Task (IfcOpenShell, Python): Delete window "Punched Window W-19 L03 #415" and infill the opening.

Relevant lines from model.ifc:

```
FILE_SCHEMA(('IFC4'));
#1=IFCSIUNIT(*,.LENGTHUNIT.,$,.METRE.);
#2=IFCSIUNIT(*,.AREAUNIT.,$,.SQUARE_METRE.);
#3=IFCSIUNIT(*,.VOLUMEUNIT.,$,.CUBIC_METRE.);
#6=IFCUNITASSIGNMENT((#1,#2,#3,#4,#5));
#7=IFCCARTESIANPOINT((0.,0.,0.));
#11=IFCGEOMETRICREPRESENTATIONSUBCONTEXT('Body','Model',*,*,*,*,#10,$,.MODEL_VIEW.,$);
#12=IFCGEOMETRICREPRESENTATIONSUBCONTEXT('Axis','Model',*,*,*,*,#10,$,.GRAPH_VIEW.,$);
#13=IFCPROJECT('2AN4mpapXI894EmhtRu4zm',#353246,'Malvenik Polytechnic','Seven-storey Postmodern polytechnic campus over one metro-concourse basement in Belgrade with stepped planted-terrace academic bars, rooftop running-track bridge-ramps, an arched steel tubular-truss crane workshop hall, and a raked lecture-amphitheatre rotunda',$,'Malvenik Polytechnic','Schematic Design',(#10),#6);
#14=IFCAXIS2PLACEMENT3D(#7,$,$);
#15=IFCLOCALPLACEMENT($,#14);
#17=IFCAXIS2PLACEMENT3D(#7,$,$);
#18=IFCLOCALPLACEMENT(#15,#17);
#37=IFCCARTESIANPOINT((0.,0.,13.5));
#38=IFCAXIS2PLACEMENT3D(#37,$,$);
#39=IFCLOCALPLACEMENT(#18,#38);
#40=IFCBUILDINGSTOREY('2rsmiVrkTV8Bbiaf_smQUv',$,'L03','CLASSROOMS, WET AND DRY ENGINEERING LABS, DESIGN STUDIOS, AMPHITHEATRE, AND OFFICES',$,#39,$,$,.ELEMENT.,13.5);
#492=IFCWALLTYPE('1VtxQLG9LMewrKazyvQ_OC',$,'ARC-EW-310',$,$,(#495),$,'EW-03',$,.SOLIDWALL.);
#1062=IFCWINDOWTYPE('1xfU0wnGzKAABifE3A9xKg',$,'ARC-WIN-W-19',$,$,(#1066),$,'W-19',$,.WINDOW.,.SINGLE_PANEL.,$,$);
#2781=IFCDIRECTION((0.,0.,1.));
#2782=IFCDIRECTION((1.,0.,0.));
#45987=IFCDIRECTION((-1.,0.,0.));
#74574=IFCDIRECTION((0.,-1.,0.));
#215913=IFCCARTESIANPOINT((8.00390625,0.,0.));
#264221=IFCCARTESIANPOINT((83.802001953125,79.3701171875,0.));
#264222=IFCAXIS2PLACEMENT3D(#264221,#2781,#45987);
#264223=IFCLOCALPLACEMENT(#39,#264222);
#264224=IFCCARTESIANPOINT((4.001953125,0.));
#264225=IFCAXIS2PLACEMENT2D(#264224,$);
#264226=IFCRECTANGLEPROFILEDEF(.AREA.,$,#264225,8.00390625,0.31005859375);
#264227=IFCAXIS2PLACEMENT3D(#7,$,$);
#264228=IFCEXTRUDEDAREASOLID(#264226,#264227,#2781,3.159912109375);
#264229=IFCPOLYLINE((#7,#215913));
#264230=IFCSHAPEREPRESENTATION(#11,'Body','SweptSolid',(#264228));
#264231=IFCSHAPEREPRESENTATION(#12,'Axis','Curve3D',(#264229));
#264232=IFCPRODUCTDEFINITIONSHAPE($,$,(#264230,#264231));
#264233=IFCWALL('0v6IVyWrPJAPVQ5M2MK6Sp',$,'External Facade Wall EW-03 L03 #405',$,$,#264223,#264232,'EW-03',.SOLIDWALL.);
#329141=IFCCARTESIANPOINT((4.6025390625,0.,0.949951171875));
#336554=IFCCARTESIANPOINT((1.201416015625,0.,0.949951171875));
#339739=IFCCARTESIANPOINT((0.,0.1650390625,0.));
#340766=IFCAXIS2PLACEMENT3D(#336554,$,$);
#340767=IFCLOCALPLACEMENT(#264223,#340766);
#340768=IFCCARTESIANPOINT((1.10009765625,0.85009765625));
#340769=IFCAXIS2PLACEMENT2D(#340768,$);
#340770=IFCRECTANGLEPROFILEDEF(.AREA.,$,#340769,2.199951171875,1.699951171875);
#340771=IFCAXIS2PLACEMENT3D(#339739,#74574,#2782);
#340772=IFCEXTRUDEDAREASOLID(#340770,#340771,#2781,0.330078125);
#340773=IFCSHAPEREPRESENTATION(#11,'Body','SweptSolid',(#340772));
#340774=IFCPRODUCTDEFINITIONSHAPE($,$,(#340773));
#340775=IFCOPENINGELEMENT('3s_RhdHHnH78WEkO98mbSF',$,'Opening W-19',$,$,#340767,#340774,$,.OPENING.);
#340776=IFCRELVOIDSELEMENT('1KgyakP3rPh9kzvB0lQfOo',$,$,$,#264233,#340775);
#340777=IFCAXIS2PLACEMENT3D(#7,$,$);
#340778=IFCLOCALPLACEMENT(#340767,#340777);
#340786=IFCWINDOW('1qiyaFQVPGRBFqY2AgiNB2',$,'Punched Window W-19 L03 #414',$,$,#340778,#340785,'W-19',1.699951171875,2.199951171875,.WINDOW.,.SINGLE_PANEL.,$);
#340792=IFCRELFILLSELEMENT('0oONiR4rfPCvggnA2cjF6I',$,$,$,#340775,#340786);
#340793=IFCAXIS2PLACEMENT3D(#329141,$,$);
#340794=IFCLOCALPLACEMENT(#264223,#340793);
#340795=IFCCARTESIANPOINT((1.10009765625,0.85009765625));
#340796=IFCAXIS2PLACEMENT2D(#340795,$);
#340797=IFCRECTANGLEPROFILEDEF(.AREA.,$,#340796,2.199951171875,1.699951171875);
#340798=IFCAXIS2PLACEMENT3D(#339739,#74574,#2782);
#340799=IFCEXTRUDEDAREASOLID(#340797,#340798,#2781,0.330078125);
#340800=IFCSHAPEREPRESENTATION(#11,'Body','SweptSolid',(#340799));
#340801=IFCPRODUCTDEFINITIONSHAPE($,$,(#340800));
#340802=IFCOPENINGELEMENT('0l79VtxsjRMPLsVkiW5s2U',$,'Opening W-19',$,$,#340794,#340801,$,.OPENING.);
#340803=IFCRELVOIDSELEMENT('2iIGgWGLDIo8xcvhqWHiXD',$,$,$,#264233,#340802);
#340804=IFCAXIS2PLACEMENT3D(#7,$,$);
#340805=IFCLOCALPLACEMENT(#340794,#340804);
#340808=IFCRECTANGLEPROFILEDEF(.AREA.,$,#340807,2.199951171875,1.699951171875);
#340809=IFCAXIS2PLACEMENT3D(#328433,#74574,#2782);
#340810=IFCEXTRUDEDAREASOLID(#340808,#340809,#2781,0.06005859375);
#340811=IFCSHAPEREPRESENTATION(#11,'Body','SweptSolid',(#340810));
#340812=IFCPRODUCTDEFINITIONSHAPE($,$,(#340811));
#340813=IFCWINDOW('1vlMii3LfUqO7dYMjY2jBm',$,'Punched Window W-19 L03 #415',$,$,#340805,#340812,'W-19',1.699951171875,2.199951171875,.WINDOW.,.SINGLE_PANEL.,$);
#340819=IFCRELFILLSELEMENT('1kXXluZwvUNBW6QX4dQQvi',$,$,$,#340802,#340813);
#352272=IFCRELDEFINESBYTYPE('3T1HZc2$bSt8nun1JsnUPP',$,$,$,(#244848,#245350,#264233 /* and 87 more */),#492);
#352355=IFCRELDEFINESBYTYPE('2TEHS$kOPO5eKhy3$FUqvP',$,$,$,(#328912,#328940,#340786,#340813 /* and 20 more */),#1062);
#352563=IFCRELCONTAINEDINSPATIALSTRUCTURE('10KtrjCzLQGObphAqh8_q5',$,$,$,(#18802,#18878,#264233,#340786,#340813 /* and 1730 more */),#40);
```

```python
import ifcopenshell
import ifcopenshell.api.feature
import ifcopenshell.api.root
import ifcopenshell.geom
import ifcopenshell.util.shape

model = ifcopenshell.open("model.ifc")
settings = ifcopenshell.geom.settings()


def volume(element):
    """Net volume in cubic metres, openings subtracted."""
    shape = ifcopenshell.geom.create_shape(settings, element)
    return ifcopenshell.util.shape.get_volume(shape.geometry)


window = model.by_id(340813)
opening = window.FillsVoids[0].RelatingOpeningElement
wall = opening.VoidsElements[0].RelatingBuildingElement
before = volume(wall)

ifcopenshell.api.root.remove_product(model, product=window)
ifcopenshell.api.feature.remove_feature(model, feature=opening)

after = volume(wall)

print(f"wall volume {before:.3f} -> {after:.3f} m3")

model.write("model_edited.ifc")
```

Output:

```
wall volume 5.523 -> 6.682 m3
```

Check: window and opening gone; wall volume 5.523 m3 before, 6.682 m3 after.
